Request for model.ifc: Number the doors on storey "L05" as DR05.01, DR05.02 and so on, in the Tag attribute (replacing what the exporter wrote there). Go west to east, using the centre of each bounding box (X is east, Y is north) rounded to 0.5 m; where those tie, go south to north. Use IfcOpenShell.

First a look at what the model holds.

```python
import ifcopenshell
import ifcopenshell.util.element
import ifcopenshell.util.placement

model = ifcopenshell.open("model.ifc")
print(model.schema)
storey = next(s for s in model.by_type("IfcBuildingStorey") if s.Name == "L05")
doors = [e for e in ifcopenshell.util.element.get_decomposition(storey) if e.is_a("IfcDoor")]
for e in sorted(doors, key=lambda e: e.id()):
    origin = ifcopenshell.util.placement.get_local_placement(e.ObjectPlacement)[:3, 3]
    print(e.id(), e.Tag, e.Name, origin.round(2) + 0.0, sep=" | ")
```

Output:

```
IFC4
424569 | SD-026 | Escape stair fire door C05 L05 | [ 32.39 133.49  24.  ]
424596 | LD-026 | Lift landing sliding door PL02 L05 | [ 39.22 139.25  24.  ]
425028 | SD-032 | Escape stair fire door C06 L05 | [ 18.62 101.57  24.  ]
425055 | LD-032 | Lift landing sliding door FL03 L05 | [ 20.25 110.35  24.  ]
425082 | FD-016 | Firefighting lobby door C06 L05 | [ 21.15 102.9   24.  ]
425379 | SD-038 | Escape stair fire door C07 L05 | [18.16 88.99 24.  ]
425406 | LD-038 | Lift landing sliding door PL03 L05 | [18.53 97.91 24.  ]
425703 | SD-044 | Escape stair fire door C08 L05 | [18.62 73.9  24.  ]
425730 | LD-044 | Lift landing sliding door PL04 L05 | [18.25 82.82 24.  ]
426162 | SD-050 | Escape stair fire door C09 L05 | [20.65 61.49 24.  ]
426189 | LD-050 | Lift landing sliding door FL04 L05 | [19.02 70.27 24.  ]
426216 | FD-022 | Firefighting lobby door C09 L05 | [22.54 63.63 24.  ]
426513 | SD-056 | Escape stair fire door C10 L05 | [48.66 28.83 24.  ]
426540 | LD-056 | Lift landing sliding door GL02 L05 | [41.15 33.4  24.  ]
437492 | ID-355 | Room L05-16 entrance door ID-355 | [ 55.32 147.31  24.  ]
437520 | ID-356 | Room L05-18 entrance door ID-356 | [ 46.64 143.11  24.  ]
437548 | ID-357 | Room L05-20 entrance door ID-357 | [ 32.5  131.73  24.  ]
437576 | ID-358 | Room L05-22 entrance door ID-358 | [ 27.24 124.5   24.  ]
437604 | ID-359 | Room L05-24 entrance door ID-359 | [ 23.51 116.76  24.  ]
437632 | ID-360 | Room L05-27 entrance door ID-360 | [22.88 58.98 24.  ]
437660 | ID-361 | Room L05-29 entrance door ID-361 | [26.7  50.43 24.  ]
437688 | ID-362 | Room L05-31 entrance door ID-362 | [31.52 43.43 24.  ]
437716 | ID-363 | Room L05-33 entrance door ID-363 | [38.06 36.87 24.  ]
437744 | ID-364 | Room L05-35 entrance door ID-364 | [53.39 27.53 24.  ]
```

```python
import ifcopenshell
import ifcopenshell.geom
import ifcopenshell.util.element
import ifcopenshell.util.shape

model = ifcopenshell.open("model.ifc")
settings = ifcopenshell.geom.settings()
settings.set("use-world-coords", True)


def centre(element):
    shape = ifcopenshell.geom.create_shape(settings, element)
    return ifcopenshell.util.shape.get_bbox_centroid(shape.geometry)


storey = next(s for s in model.by_type("IfcBuildingStorey") if s.Name == "L05")
doors = [e for e in ifcopenshell.util.element.get_decomposition(storey) if e.is_a("IfcDoor")]

# Insertion points can sit at a corner or the storey origin, so sort by the geometry (in metres).
centres = {e: centre(e) for e in doors}
doors.sort(key=lambda e: (round(centres[e][0] / 0.5), centres[e][1]))

for i, e in enumerate(doors, start=1):
    number = f"DR05.{i:02d}"
    e.Tag = number
    print(e.id(), number)

model.write("model_updated.ifc")
```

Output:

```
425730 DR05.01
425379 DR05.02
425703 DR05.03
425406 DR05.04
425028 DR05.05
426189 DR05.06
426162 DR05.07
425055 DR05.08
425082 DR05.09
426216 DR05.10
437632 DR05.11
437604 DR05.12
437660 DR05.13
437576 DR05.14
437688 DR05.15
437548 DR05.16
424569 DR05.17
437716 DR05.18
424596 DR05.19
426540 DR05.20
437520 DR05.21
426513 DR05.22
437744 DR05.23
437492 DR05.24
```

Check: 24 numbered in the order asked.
